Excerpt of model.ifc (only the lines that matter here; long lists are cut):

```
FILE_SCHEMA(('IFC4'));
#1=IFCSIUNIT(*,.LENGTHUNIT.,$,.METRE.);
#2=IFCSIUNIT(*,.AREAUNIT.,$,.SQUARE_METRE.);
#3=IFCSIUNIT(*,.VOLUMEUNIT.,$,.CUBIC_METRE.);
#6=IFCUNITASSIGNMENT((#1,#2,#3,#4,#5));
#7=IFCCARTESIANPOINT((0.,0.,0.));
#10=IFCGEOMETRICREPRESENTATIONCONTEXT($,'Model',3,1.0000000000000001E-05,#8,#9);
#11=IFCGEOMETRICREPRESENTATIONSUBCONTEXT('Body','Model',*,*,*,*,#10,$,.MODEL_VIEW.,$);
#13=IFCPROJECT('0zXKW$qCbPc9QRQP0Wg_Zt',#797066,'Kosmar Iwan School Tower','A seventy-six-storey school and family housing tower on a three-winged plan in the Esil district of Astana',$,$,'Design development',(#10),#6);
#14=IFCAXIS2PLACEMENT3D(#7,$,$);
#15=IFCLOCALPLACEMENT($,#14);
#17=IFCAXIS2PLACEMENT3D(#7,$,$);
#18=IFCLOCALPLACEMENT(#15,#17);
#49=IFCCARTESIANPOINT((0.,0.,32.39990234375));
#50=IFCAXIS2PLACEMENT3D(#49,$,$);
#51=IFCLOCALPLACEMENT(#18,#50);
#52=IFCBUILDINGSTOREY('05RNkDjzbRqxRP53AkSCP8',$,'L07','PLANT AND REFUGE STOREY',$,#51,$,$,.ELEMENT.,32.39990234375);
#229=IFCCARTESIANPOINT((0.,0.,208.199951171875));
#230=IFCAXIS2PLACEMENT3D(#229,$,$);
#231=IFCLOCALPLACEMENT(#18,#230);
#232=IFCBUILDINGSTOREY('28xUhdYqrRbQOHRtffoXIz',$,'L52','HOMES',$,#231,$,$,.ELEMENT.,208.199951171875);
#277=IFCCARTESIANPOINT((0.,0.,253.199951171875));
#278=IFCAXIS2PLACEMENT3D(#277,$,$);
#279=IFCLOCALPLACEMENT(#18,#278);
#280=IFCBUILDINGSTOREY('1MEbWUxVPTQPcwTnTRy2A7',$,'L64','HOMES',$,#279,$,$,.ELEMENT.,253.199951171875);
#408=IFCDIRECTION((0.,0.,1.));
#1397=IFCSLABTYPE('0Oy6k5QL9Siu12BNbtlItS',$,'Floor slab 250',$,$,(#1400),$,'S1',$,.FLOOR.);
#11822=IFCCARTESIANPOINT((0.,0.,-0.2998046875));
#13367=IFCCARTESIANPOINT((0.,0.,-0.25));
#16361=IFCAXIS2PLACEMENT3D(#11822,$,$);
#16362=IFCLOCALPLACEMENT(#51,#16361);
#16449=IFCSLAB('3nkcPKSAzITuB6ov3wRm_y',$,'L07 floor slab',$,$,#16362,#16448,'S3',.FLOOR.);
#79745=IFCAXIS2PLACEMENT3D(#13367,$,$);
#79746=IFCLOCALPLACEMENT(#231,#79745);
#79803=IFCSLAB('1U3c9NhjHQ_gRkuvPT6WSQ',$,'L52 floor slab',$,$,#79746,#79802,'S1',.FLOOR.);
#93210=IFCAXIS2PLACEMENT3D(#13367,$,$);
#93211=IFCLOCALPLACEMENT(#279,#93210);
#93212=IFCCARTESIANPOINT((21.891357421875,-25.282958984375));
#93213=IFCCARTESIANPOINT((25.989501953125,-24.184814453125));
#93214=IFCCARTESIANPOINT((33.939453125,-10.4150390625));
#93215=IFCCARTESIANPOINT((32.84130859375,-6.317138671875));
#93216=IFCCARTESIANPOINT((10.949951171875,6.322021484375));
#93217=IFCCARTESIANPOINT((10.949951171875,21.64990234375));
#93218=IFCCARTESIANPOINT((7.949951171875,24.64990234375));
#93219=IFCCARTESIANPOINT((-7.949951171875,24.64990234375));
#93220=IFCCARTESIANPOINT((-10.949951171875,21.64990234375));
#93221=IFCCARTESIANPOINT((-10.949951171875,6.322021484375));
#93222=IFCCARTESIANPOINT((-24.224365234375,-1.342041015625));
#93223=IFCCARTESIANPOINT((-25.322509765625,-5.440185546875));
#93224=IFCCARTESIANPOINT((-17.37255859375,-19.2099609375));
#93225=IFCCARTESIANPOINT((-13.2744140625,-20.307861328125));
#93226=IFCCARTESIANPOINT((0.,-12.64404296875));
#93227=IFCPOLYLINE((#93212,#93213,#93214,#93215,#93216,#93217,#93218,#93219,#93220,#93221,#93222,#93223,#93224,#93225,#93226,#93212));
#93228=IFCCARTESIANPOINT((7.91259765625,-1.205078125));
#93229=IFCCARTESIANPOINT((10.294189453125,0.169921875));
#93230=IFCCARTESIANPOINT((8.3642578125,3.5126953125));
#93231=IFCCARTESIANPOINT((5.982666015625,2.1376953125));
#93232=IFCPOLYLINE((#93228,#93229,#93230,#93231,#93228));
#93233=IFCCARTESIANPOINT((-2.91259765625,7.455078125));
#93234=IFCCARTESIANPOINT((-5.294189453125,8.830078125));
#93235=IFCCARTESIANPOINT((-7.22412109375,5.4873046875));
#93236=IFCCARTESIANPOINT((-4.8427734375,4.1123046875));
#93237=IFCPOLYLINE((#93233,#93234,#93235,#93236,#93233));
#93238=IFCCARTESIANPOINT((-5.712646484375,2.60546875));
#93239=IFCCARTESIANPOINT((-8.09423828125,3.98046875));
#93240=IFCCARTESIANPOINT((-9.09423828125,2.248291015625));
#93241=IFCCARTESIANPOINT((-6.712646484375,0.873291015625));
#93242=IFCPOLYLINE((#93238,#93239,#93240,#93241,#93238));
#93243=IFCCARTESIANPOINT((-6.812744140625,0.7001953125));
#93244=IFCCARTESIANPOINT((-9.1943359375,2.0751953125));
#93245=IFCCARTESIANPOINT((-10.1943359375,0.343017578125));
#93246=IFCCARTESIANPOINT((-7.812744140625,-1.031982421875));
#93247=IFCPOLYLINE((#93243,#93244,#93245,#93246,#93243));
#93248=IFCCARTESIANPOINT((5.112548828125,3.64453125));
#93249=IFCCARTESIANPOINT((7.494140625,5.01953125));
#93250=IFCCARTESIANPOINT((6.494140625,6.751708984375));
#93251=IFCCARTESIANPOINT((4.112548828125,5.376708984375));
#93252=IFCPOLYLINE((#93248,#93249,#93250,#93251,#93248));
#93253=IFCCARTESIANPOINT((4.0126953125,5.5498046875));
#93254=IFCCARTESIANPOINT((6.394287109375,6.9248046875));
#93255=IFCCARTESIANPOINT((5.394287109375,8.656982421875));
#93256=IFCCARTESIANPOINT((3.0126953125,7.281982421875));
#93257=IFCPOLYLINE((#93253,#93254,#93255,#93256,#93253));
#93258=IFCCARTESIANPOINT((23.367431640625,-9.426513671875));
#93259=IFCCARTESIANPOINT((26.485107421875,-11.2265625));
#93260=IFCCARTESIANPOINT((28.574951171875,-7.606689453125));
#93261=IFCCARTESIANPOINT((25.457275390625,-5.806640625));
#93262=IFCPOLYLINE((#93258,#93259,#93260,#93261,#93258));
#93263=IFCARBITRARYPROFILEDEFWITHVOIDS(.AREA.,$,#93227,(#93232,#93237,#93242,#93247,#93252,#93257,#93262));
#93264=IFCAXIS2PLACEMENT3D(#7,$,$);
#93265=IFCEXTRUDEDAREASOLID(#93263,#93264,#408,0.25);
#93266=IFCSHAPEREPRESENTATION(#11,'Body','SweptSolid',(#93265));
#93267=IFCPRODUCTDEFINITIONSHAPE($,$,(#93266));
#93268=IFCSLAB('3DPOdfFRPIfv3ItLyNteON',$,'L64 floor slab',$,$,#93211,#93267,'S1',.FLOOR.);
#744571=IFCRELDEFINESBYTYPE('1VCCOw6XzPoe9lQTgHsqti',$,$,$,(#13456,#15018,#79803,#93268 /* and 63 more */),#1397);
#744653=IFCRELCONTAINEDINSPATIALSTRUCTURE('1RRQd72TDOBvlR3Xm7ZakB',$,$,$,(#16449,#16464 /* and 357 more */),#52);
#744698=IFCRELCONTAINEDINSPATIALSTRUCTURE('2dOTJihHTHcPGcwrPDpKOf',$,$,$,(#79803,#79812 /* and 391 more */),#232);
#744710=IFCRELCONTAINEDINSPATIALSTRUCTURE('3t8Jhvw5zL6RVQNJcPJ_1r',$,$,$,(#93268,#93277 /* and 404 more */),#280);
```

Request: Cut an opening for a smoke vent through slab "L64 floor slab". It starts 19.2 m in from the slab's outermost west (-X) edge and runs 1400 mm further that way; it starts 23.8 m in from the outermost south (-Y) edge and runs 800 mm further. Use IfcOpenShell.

```python
import numpy as np
import ifcopenshell
import ifcopenshell.api.feature
import ifcopenshell.api.geometry
import ifcopenshell.api.root
import ifcopenshell.geom
import ifcopenshell.util.placement
import ifcopenshell.util.representation
import ifcopenshell.util.shape
import ifcopenshell.util.unit

model = ifcopenshell.open("model.ifc")
unit_scale = ifcopenshell.util.unit.calculate_unit_scale(model)
settings = ifcopenshell.geom.settings()


def volume(element):
    """Net volume in cubic metres, openings subtracted."""
    shape = ifcopenshell.geom.create_shape(settings, element)
    return ifcopenshell.util.shape.get_volume(shape.geometry)


slab = model.by_guid("3DPOdfFRPIfv3ItLyNteON")
before = volume(slab)

# Extent in the slab's own axes, in metres. The edges named are its -X and -Y sides.
slab_shape = ifcopenshell.geom.create_shape(settings, slab)
vertices = ifcopenshell.util.shape.get_vertices(slab_shape.geometry)
x_min, y_min, bottom = vertices.min(axis=0)
top = vertices[:, 2].max()

opening = ifcopenshell.api.root.create_entity(model, ifc_class="IfcOpeningElement", name="Smoke vent opening", predefined_type="OPENING")
context = ifcopenshell.util.representation.get_context(model, "Model", "Body", "MODEL_VIEW")
width, depth = 1.4, 0.8
outline = [(0.0, 0.0), (width, 0.0), (width, depth), (0.0, depth), (0.0, 0.0)]
# Overshoot both faces by 50 mm so the cut is clean.
shape = ifcopenshell.api.geometry.add_slab_representation(
    model, context=context, depth=top - bottom + 0.1, polyline=outline
)
ifcopenshell.api.geometry.assign_representation(model, product=opening, representation=shape)

matrix = ifcopenshell.util.placement.get_local_placement(slab.ObjectPlacement)
matrix[:, 3] = matrix @ np.append(np.array([x_min + 19.2, y_min + 23.8, bottom - 0.05]) / unit_scale, 1.0)
ifcopenshell.api.geometry.edit_object_placement(model, product=opening, matrix=matrix, is_si=False)
ifcopenshell.api.feature.add_feature(model, feature=opening, element=slab)

after = volume(slab)

print(f"slab volume {before:.3f} -> {after:.3f} m3")

model.write("model_rev.ifc")
```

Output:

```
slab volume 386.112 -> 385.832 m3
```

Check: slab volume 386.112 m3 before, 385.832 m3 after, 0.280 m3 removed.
